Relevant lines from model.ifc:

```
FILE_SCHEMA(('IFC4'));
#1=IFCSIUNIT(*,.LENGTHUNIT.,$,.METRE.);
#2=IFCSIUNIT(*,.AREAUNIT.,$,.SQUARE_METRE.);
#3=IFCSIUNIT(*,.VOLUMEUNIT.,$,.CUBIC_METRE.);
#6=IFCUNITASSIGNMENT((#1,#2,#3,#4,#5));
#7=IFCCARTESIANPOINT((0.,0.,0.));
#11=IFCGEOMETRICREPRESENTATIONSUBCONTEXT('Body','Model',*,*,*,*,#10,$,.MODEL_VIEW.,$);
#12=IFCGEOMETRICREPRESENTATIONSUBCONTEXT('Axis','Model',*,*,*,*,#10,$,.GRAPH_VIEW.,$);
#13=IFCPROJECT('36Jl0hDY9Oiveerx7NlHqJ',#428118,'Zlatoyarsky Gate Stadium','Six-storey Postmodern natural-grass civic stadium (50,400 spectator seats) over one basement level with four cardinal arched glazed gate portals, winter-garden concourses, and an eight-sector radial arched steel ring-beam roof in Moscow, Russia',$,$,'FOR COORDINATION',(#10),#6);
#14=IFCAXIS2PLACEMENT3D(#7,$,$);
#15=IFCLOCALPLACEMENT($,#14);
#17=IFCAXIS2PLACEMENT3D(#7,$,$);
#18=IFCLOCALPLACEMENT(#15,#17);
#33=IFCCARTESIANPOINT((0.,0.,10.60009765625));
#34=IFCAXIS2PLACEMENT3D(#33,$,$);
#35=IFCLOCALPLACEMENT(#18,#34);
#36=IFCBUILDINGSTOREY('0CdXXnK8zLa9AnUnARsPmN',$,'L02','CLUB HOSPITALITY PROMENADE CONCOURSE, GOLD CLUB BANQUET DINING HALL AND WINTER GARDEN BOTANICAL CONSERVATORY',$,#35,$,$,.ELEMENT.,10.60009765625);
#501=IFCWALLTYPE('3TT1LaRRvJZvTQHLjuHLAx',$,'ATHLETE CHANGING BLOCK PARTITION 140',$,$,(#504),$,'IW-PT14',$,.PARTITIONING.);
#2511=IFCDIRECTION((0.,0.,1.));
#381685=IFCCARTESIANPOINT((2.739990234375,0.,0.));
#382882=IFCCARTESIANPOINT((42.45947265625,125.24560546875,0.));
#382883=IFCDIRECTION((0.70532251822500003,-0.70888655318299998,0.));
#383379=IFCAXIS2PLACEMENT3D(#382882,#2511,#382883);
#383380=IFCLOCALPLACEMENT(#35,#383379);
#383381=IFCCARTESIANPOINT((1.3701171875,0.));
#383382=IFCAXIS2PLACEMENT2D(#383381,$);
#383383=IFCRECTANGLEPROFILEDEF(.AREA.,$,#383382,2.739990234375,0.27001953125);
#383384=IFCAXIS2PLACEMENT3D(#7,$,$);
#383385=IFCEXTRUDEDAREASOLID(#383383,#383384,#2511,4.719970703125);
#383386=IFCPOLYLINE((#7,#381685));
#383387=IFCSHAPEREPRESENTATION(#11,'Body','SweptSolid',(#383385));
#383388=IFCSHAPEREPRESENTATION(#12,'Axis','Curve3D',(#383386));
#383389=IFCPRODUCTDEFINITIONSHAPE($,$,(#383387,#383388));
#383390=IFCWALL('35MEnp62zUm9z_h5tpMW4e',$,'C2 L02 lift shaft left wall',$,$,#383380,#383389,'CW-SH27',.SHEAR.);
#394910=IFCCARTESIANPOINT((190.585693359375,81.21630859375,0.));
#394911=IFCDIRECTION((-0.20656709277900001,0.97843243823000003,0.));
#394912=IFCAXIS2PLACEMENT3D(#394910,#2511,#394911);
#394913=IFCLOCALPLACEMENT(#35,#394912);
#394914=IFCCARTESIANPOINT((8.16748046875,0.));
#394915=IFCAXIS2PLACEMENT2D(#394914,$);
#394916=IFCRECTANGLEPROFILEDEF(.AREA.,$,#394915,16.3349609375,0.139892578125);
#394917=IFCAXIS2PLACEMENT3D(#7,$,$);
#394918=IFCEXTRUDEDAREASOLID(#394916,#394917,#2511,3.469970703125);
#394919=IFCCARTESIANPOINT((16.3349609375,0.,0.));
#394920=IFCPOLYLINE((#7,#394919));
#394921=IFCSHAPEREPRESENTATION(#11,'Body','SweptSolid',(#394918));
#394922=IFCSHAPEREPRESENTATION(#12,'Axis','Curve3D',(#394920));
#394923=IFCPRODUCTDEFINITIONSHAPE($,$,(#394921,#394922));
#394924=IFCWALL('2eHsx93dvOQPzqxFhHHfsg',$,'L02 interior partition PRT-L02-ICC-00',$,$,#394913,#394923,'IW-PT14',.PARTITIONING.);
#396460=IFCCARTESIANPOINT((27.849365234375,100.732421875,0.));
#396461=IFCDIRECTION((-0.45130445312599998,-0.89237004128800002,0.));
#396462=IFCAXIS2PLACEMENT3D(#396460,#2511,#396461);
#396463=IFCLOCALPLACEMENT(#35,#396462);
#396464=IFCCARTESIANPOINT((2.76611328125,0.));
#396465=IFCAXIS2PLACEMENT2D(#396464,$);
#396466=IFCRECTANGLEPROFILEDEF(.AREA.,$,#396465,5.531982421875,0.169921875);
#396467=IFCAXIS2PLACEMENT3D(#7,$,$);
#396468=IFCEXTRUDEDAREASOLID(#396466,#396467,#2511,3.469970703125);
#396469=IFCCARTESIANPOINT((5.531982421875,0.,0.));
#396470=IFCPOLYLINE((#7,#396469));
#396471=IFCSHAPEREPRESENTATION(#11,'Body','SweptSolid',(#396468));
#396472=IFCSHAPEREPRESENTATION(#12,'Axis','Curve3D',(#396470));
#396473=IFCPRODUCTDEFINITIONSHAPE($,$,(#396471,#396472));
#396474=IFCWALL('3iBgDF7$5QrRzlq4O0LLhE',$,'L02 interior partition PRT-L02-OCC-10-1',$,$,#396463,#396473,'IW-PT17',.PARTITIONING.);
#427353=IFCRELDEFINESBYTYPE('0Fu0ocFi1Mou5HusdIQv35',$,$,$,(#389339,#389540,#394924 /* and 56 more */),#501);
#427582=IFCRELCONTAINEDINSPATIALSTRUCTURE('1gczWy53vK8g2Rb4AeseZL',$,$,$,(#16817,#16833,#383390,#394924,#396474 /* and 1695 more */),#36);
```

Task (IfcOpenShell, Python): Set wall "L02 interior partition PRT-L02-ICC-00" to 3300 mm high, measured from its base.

```python
import ifcopenshell
import ifcopenshell.geom
import ifcopenshell.util.representation
import ifcopenshell.util.shape
import ifcopenshell.util.unit

model = ifcopenshell.open("model.ifc")
unit_scale = ifcopenshell.util.unit.calculate_unit_scale(model)
settings = ifcopenshell.geom.settings()


def volume(element):
    """Net volume in cubic metres, openings subtracted."""
    shape = ifcopenshell.geom.create_shape(settings, element)
    return ifcopenshell.util.shape.get_volume(shape.geometry)


wall = model.by_guid("2eHsx93dvOQPzqxFhHHfsg")
before = volume(wall)

body = ifcopenshell.util.representation.get_representation(wall, "Model", "Body")
solid = body.Items[0]
old_height = solid.Depth
solid.Depth = 3.3 / unit_scale
after = volume(wall)

print(f"height {old_height:g} -> {solid.Depth:g}, volume {before:.3f} -> {after:.3f} m3")

model.write("model_v2.ifc")
```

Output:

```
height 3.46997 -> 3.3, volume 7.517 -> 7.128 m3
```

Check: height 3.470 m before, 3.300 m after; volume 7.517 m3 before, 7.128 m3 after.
